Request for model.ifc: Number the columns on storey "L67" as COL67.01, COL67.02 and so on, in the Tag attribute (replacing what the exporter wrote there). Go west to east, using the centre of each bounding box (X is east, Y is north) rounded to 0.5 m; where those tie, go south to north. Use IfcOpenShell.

First a look at what the model holds.

```python
import ifcopenshell
import ifcopenshell.util.element
import ifcopenshell.util.placement

model = ifcopenshell.open("model.ifc")
print(model.schema)
storey = next(s for s in model.by_type("IfcBuildingStorey") if s.Name == "L67")
columns = [e for e in ifcopenshell.util.element.get_decomposition(storey) if e.is_a("IfcColumn")]
for e in sorted(columns, key=lambda e: e.id()):
    origin = ifcopenshell.util.placement.get_local_placement(e.ObjectPlacement)[:3, 3]
    print(e.id(), e.Tag, e.Name, origin.round(2) + 0.0, sep=" | ")
```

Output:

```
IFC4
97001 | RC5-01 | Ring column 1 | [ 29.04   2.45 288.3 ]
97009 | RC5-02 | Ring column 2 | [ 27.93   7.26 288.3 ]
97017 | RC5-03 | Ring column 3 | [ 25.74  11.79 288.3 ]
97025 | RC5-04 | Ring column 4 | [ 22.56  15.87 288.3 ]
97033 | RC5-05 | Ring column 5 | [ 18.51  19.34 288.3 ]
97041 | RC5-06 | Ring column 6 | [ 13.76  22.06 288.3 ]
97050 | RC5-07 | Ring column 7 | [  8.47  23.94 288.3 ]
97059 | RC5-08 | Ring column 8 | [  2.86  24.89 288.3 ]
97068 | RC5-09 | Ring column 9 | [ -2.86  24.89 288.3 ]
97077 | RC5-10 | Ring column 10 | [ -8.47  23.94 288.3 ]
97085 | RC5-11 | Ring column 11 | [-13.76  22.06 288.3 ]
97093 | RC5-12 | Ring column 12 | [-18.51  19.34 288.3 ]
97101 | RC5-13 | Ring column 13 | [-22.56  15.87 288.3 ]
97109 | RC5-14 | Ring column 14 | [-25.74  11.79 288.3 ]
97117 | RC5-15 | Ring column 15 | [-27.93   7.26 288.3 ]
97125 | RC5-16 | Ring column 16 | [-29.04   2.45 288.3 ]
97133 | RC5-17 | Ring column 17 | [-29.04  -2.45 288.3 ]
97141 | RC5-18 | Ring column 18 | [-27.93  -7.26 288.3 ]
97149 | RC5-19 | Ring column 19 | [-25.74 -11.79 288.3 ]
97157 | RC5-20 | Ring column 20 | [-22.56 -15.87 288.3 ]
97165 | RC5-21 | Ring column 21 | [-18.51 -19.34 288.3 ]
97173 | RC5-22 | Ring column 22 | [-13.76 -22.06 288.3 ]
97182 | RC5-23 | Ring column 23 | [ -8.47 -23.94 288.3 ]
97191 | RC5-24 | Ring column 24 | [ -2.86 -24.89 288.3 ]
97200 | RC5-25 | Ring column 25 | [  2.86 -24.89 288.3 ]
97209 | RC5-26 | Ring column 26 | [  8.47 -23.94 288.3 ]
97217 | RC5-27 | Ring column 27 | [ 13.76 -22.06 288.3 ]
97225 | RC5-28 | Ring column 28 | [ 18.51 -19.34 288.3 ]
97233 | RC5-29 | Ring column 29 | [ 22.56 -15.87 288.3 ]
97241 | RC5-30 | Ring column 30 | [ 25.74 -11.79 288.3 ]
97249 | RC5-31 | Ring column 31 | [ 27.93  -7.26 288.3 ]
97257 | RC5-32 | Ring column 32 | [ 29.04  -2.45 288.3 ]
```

```python
import ifcopenshell
import ifcopenshell.geom
import ifcopenshell.util.element
import ifcopenshell.util.shape

model = ifcopenshell.open("model.ifc")
settings = ifcopenshell.geom.settings()
settings.set("use-world-coords", True)


def centre(element):
    shape = ifcopenshell.geom.create_shape(settings, element)
    return ifcopenshell.util.shape.get_bbox_centroid(shape.geometry)


storey = next(s for s in model.by_type("IfcBuildingStorey") if s.Name == "L67")
columns = [e for e in ifcopenshell.util.element.get_decomposition(storey) if e.is_a("IfcColumn")]

# Insertion points can sit at a corner or the storey origin, so sort by the geometry (in metres).
centres = {e: centre(e) for e in columns}
columns.sort(key=lambda e: (round(centres[e][0] / 0.5), centres[e][1]))

for i, e in enumerate(columns, start=1):
    number = f"COL67.{i:02d}"
    e.Tag = number
    print(e.id(), number)

model.write("model_rev.ifc")
```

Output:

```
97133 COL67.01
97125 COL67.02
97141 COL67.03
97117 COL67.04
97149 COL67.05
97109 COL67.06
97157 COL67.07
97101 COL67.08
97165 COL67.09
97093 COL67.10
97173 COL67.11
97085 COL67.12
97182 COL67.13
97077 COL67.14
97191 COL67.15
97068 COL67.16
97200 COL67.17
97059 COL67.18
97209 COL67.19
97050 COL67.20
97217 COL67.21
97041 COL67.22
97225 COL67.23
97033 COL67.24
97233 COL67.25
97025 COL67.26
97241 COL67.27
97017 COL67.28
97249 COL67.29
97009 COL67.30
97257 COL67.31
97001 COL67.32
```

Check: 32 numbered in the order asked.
